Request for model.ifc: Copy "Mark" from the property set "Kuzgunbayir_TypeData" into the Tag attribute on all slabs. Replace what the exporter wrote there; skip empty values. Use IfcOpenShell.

First a look at what the model holds.

```python
import ifcopenshell
import ifcopenshell.util.element

model = ifcopenshell.open("model.ifc")
print(model.schema)
slabs = model.by_type("IfcSlab")
print(len(slabs), "slabs")
for e in slabs[:8]:
    source = ifcopenshell.util.element.get_pset(e, "Kuzgunbayir_TypeData", "Mark")
    target = e.Tag
    print(e.id(), repr(source), repr(target), sep=" | ")
```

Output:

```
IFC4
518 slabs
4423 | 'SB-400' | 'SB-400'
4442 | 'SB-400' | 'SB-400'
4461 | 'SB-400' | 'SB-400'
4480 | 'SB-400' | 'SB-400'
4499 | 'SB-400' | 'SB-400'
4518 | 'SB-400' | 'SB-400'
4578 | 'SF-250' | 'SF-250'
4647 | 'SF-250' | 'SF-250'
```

```python
import ifcopenshell
import ifcopenshell.util.element

model = ifcopenshell.open("model.ifc")

count = 0
for e in model.by_type("IfcSlab"):
    value = ifcopenshell.util.element.get_pset(e, "Kuzgunbayir_TypeData", "Mark")
    current = e.Tag
    if not value or not value.strip() or current == value:
        continue
    e.Tag = value
    count += 1

print(count, "slabs updated")

model.write("model_rev.ifc")
```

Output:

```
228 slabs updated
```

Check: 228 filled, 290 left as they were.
